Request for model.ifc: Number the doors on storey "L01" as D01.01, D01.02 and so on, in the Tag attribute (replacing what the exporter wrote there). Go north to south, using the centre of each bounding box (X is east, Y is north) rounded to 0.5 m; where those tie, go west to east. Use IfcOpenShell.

First a look at what the model holds.

```python
import ifcopenshell
import ifcopenshell.util.element
import ifcopenshell.util.placement

model = ifcopenshell.open("model.ifc")
print(model.schema)
storey = next(s for s in model.by_type("IfcBuildingStorey") if s.Name == "L01")
doors = [e for e in ifcopenshell.util.element.get_decomposition(storey) if e.is_a("IfcDoor")]
for e in sorted(doors, key=lambda e: e.id()):
    origin = ifcopenshell.util.placement.get_local_placement(e.ObjectPlacement)[:3, 3]
    print(e.id(), e.Tag, e.Name, origin.round(2) + 0.0, sep=" | ")
```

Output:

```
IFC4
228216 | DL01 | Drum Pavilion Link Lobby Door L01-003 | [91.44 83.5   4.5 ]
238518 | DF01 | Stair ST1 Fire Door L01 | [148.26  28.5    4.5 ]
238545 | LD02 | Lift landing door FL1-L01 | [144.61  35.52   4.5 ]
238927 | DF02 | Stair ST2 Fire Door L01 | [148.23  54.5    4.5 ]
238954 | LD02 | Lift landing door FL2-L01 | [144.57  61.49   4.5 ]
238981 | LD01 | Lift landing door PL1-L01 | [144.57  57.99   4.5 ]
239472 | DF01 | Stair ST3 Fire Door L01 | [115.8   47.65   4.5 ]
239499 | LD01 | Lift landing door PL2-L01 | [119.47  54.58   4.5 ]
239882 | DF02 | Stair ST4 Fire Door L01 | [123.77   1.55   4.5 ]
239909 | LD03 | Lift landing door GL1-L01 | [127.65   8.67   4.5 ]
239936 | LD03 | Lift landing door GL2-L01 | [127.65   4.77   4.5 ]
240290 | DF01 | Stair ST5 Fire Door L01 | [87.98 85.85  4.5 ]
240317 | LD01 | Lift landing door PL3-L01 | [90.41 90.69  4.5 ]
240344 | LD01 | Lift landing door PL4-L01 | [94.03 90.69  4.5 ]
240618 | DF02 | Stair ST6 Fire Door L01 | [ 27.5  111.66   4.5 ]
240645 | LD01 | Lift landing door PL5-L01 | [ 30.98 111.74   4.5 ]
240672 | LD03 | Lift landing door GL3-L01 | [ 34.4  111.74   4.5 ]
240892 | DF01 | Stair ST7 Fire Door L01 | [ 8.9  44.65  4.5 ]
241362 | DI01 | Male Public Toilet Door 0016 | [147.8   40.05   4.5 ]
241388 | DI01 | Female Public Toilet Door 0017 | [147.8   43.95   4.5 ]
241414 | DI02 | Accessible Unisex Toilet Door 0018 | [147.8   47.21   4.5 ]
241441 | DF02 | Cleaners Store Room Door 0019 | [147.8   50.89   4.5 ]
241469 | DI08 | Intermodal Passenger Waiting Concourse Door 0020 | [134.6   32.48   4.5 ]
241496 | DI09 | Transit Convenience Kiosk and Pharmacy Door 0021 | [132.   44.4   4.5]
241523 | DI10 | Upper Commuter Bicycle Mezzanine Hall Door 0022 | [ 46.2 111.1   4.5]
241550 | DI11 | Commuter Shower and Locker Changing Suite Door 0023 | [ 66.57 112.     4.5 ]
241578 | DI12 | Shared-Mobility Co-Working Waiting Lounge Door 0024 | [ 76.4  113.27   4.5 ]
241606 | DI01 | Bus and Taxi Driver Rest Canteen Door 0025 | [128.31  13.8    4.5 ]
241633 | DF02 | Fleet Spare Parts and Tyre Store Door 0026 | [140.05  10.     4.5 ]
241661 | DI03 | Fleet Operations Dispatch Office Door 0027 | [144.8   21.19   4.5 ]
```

```python
import ifcopenshell
import ifcopenshell.geom
import ifcopenshell.util.element
import ifcopenshell.util.shape

model = ifcopenshell.open("model.ifc")
settings = ifcopenshell.geom.settings()
settings.set("use-world-coords", True)


def centre(element):
    shape = ifcopenshell.geom.create_shape(settings, element)
    return ifcopenshell.util.shape.get_bbox_centroid(shape.geometry)


storey = next(s for s in model.by_type("IfcBuildingStorey") if s.Name == "L01")
doors = [e for e in ifcopenshell.util.element.get_decomposition(storey) if e.is_a("IfcDoor")]

# Insertion points can sit at a corner or the storey origin, so sort by the geometry (in metres).
centres = {e: centre(e) for e in doors}
doors.sort(key=lambda e: (-round(centres[e][1] / 0.5), centres[e][0]))

for i, e in enumerate(doors, start=1):
    number = f"D01.{i:02d}"
    e.Tag = number
    print(e.id(), number)

model.write("model_edited.ifc")
```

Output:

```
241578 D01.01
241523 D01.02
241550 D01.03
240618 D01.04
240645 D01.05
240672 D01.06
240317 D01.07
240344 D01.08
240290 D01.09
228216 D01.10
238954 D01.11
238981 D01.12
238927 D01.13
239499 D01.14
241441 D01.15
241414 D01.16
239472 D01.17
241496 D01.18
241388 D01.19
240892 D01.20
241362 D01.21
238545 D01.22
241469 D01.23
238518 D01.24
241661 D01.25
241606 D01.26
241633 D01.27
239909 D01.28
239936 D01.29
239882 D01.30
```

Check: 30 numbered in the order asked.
